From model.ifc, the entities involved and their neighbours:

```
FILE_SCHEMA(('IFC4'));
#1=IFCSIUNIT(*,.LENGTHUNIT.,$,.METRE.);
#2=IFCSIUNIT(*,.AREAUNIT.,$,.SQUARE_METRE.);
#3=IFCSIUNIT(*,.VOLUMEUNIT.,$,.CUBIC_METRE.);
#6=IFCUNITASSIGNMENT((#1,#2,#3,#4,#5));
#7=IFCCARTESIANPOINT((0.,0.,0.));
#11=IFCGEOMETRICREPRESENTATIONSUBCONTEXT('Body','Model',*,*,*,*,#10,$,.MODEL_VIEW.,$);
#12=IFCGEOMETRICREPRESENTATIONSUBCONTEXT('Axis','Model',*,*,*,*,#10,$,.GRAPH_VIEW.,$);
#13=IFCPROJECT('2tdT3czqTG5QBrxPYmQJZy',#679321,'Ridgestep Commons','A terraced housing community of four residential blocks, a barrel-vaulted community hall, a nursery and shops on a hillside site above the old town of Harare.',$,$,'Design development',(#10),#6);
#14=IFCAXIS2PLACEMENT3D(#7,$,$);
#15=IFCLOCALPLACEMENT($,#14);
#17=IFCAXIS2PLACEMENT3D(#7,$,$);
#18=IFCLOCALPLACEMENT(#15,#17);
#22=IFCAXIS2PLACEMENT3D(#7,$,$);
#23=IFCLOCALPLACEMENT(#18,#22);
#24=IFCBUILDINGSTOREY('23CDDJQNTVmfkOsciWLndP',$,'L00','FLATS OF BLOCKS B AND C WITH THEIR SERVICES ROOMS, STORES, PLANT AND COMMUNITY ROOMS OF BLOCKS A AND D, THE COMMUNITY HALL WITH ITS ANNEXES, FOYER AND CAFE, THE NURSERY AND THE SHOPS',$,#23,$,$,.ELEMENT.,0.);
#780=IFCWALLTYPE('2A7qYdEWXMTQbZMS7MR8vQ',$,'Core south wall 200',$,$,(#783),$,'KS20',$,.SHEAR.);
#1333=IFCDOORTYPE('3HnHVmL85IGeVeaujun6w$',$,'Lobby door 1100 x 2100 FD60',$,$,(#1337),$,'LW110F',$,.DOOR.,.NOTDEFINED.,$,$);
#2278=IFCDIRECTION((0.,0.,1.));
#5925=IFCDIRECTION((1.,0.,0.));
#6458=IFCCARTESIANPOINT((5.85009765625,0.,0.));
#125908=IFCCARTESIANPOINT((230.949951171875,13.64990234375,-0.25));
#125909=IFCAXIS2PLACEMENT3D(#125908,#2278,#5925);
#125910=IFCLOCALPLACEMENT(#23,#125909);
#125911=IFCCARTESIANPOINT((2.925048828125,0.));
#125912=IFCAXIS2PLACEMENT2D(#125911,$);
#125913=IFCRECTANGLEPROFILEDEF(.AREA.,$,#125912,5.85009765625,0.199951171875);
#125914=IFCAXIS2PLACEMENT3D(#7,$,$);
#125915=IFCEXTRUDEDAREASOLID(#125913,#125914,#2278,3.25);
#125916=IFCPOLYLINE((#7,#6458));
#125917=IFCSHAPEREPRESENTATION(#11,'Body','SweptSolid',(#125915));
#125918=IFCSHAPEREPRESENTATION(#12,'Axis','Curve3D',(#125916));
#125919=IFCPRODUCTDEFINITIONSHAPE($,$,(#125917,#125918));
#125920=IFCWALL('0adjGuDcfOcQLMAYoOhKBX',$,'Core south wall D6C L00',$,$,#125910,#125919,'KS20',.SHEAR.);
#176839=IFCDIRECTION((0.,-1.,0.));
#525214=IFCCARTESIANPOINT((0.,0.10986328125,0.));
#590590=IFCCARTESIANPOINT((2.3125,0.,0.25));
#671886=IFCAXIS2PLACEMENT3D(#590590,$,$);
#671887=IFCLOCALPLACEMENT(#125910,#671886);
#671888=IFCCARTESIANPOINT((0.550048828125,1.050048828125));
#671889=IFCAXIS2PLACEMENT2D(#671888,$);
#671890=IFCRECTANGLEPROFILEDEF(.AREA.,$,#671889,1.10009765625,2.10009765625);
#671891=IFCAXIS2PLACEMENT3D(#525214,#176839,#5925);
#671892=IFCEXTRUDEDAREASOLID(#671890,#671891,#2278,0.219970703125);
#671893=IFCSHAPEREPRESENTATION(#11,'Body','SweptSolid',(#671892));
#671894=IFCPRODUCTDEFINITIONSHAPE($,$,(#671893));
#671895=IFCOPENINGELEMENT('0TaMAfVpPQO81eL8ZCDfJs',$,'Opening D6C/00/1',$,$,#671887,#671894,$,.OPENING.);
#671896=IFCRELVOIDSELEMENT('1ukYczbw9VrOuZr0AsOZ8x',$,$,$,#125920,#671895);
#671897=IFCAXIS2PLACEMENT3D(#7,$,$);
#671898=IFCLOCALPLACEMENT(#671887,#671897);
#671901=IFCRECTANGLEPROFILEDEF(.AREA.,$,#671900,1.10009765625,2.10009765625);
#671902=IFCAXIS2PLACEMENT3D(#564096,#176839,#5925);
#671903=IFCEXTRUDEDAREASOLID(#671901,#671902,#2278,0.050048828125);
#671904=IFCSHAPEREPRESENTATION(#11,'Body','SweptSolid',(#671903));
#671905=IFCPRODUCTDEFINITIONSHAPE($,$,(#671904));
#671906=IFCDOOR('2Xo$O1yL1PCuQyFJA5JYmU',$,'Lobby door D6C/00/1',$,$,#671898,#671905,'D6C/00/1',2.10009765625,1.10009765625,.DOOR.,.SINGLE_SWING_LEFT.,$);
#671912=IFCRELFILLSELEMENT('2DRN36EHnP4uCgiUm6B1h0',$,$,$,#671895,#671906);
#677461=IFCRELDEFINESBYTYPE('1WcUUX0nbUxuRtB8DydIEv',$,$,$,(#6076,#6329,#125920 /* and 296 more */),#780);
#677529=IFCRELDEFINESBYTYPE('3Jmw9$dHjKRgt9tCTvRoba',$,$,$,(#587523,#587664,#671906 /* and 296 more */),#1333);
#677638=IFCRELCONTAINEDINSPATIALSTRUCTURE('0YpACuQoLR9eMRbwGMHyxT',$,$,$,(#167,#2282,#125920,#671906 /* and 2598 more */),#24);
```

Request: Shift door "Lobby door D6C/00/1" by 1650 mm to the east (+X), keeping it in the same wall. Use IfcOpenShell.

```python
import ifcopenshell
import ifcopenshell.api.geometry
import ifcopenshell.util.placement
import ifcopenshell.util.unit

model = ifcopenshell.open("model.ifc")
unit_scale = ifcopenshell.util.unit.calculate_unit_scale(model)

door = model.by_guid("2Xo$O1yL1PCuQyFJA5JYmU")
opening = door.FillsVoids[0].RelatingOpeningElement
wall = opening.VoidsElements[0].RelatingBuildingElement

wall_matrix = ifcopenshell.util.placement.get_local_placement(wall.ObjectPlacement)
shift = wall_matrix[:3, 0] * 1.65 / unit_scale
before = ifcopenshell.util.placement.get_local_placement(door.ObjectPlacement)[:3, 3].copy()

# The door is placed relative to its opening, so it follows when the opening moves.
matrix = ifcopenshell.util.placement.get_local_placement(opening.ObjectPlacement)
matrix[:3, 3] += shift
ifcopenshell.api.geometry.edit_object_placement(
    model, product=opening, matrix=matrix, is_si=False, should_transform_children=True
)

after = ifcopenshell.util.placement.get_local_placement(door.ObjectPlacement)[:3, 3]
print("door moved by", (after - before).round(3) + 0.0)

model.write("model-out.ifc")
```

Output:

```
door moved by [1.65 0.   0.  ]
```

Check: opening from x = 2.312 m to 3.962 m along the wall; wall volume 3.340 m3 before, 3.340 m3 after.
